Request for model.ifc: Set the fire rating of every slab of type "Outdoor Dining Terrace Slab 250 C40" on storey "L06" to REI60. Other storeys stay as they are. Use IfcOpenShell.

First a look at what the model holds.

```python
import ifcopenshell
import ifcopenshell.util.element

model = ifcopenshell.open("model.ifc")
print(model.schema)
storey = next(s for s in model.by_type("IfcBuildingStorey") if s.Name == "L06")
slabs = [e for e in ifcopenshell.util.element.get_decomposition(storey) if e.is_a("IfcSlab")]
seen = {}
for e in slabs:
    element_type = ifcopenshell.util.element.get_type(e)
    key = (element_type.Name if element_type != e and element_type else None, ifcopenshell.util.element.get_pset(e, "Pset_SlabCommon", "FireRating"))
    seen[key] = seen.get(key, 0) + 1
for (name, value), count in sorted(seen.items(), key=str):
    print(count, "x", name, "|", value)
```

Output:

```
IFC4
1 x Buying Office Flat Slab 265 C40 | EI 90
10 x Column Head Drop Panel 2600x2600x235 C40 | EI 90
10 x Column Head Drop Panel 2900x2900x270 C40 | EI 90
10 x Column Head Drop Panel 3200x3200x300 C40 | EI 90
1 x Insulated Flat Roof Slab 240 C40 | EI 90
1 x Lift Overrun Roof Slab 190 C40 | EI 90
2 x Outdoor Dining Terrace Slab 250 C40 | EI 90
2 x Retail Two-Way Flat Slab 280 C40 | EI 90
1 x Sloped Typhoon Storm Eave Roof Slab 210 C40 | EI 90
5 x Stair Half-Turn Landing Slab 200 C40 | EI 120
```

```python
import ifcopenshell
import ifcopenshell.api.pset
import ifcopenshell.util.element

model = ifcopenshell.open("model.ifc")

storey = next(s for s in model.by_type("IfcBuildingStorey") if s.Name == "L06")
slabs = [e for e in ifcopenshell.util.element.get_decomposition(storey) if e.is_a("IfcSlab")]

count = 0
for e in slabs:
    element_type = ifcopenshell.util.element.get_type(e)
    if element_type in (None, e) or element_type.Name != "Outdoor Dining Terrace Slab 250 C40":
        continue
    # add_pset returns the element's existing set when there is one.
    pset = ifcopenshell.api.pset.add_pset(model, product=e, name="Pset_SlabCommon")
    ifcopenshell.api.pset.edit_pset(model, pset=pset, properties={"FireRating": "REI60"})
    count += 1

print(count, "slabs updated")

model.write("model-out.ifc")
```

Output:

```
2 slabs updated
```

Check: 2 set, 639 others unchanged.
